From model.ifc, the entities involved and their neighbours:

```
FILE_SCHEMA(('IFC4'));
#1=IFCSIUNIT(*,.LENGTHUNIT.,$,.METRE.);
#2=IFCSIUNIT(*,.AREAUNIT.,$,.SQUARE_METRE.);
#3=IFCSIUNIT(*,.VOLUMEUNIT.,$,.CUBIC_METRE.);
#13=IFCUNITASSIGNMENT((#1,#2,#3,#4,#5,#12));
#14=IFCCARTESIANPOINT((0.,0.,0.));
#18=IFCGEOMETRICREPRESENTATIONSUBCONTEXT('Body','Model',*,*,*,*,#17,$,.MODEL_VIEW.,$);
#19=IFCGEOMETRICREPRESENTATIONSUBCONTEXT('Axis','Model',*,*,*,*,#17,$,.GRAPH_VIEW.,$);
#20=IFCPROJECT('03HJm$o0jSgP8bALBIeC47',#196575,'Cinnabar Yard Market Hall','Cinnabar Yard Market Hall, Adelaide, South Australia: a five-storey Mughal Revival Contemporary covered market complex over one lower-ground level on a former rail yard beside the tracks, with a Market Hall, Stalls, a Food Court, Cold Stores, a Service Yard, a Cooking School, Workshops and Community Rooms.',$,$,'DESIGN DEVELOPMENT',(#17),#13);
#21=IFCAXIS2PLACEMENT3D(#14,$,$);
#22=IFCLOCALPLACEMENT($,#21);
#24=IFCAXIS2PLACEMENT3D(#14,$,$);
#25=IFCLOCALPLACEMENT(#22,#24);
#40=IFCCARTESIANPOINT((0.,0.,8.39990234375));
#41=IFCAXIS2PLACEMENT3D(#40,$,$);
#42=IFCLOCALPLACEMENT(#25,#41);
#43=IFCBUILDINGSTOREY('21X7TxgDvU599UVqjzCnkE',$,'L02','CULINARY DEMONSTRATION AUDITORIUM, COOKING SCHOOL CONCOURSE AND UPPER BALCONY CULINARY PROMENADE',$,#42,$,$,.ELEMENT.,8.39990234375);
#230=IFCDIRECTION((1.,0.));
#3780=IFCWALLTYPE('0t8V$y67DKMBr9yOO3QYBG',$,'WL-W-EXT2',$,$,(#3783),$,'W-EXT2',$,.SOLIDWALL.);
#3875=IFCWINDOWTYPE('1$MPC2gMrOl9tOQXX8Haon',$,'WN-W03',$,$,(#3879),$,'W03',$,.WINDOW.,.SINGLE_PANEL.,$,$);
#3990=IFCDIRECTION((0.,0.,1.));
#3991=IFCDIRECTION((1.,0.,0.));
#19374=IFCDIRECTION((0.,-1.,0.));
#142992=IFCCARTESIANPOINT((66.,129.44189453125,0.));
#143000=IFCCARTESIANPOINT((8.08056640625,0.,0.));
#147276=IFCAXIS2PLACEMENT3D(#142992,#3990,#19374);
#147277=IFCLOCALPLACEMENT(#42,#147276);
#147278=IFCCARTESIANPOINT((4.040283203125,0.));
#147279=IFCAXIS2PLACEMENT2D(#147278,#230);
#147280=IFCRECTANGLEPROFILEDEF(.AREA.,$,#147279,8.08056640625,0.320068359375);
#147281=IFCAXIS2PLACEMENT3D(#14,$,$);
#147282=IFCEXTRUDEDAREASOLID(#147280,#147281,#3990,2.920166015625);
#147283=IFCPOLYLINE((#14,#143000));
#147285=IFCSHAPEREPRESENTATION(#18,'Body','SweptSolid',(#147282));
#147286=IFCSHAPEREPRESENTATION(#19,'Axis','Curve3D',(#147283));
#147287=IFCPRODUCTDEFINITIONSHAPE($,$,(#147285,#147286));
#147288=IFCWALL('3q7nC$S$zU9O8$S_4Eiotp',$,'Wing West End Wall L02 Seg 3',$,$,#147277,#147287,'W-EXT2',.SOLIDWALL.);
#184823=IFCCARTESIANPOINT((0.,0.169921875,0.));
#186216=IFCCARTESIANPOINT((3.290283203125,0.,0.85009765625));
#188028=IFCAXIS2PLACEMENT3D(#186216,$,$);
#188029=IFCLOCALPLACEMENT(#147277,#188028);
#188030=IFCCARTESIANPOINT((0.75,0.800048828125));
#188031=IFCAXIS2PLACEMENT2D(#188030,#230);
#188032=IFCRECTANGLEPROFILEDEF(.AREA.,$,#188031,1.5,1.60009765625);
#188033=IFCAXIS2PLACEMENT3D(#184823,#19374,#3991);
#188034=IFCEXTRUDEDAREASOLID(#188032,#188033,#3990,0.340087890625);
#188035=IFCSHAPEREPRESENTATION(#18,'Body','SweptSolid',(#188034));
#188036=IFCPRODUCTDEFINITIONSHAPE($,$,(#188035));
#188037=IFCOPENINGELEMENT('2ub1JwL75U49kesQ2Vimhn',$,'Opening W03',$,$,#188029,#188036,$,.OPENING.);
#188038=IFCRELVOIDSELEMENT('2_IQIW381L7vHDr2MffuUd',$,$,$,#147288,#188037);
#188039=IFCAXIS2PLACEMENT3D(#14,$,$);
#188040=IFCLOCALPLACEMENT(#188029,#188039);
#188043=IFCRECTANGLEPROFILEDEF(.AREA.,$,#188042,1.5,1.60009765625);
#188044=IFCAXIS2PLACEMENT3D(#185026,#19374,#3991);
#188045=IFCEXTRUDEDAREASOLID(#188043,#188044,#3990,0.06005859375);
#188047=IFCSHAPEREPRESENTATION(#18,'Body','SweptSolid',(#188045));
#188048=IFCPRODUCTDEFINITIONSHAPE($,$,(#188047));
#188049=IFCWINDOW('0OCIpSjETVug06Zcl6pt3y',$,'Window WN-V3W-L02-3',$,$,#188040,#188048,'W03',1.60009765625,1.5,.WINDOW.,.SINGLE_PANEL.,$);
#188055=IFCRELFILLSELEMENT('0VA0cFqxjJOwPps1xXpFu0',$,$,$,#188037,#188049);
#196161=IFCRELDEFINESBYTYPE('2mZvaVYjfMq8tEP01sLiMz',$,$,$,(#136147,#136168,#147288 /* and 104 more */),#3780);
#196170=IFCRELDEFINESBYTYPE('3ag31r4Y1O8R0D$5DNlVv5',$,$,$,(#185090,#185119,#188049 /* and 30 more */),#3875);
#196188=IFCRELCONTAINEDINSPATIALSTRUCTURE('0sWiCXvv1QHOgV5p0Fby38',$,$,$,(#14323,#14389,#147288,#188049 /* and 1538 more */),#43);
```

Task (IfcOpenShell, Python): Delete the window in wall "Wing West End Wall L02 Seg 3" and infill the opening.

```python
import ifcopenshell
import ifcopenshell.api.feature
import ifcopenshell.api.root
import ifcopenshell.geom
import ifcopenshell.util.shape

model = ifcopenshell.open("model.ifc")
settings = ifcopenshell.geom.settings()


def volume(element):
    """Net volume in cubic metres, openings subtracted."""
    shape = ifcopenshell.geom.create_shape(settings, element)
    return ifcopenshell.util.shape.get_volume(shape.geometry)


window = model.by_guid("0OCIpSjETVug06Zcl6pt3y")
opening = window.FillsVoids[0].RelatingOpeningElement
wall = opening.VoidsElements[0].RelatingBuildingElement
before = volume(wall)

ifcopenshell.api.root.remove_product(model, product=window)
ifcopenshell.api.feature.remove_feature(model, feature=opening)

after = volume(wall)

print(f"wall volume {before:.3f} -> {after:.3f} m3")

model.write("model_v2.ifc")
```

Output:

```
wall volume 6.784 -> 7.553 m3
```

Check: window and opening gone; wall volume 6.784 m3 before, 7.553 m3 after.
